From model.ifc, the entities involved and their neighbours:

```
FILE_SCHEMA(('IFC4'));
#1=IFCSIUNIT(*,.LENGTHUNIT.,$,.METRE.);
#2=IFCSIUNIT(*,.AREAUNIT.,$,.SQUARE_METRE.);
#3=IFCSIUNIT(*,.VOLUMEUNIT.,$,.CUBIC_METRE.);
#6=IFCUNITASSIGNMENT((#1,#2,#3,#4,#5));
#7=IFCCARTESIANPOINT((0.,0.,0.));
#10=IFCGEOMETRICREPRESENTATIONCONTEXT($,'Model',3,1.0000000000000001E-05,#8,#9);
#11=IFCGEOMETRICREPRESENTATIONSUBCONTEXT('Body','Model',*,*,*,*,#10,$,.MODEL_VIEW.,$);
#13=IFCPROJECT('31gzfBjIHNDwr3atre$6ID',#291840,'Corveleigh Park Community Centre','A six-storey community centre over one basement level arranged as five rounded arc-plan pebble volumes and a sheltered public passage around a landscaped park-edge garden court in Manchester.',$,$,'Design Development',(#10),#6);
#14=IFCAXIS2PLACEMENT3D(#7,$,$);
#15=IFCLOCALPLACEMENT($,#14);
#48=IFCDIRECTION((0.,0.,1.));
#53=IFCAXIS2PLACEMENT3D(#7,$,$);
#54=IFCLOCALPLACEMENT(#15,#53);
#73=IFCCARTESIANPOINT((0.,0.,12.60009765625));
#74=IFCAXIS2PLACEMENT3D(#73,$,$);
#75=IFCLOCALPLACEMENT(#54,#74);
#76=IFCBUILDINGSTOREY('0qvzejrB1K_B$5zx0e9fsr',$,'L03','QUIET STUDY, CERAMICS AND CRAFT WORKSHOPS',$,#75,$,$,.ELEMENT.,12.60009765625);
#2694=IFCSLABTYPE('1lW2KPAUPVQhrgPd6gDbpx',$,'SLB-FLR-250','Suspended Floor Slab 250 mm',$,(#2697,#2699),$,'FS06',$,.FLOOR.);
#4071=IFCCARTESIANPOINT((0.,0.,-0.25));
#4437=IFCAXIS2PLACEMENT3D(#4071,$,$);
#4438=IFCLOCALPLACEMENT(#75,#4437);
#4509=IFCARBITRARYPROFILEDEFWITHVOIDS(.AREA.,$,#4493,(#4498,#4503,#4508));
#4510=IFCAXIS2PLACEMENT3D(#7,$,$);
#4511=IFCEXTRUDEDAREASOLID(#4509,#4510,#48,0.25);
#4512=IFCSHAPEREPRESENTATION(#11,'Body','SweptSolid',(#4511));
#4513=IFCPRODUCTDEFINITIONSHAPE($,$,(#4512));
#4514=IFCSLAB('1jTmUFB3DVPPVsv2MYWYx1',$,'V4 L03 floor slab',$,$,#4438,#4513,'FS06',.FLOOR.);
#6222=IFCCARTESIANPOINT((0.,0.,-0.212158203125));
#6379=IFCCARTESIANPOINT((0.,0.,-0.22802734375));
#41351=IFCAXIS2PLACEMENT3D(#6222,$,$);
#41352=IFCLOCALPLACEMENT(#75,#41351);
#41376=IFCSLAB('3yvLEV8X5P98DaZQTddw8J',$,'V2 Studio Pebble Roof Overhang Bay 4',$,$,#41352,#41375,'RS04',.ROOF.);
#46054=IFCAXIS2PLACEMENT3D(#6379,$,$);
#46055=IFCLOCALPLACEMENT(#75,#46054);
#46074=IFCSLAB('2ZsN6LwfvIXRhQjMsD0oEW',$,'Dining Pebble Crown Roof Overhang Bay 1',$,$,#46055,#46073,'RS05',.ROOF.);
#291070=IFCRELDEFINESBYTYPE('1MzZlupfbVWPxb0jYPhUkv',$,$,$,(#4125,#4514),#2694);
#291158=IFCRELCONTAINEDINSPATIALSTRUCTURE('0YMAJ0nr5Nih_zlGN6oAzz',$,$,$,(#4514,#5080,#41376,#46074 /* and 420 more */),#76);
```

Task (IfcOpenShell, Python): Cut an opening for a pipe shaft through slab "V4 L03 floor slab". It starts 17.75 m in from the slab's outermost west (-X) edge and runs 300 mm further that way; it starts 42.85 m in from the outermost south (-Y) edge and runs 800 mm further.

```python
import numpy as np
import ifcopenshell
import ifcopenshell.api.feature
import ifcopenshell.api.geometry
import ifcopenshell.api.root
import ifcopenshell.geom
import ifcopenshell.util.placement
import ifcopenshell.util.representation
import ifcopenshell.util.shape
import ifcopenshell.util.unit

model = ifcopenshell.open("model.ifc")
unit_scale = ifcopenshell.util.unit.calculate_unit_scale(model)
settings = ifcopenshell.geom.settings()


def volume(element):
    """Net volume in cubic metres, openings subtracted."""
    shape = ifcopenshell.geom.create_shape(settings, element)
    return ifcopenshell.util.shape.get_volume(shape.geometry)


slab = model.by_guid("1jTmUFB3DVPPVsv2MYWYx1")
before = volume(slab)

# Extent in the slab's own axes, in metres. The edges named are its -X and -Y sides.
slab_shape = ifcopenshell.geom.create_shape(settings, slab)
vertices = ifcopenshell.util.shape.get_vertices(slab_shape.geometry)
x_min, y_min, bottom = vertices.min(axis=0)
top = vertices[:, 2].max()

opening = ifcopenshell.api.root.create_entity(model, ifc_class="IfcOpeningElement", name="Pipe shaft opening", predefined_type="OPENING")
context = ifcopenshell.util.representation.get_context(model, "Model", "Body", "MODEL_VIEW")
width, depth = 0.3, 0.8
outline = [(0.0, 0.0), (width, 0.0), (width, depth), (0.0, depth), (0.0, 0.0)]
# Overshoot both faces by 50 mm so the cut is clean.
shape = ifcopenshell.api.geometry.add_slab_representation(
    model, context=context, depth=top - bottom + 0.1, polyline=outline
)
ifcopenshell.api.geometry.assign_representation(model, product=opening, representation=shape)

matrix = ifcopenshell.util.placement.get_local_placement(slab.ObjectPlacement)
matrix[:, 3] = matrix @ np.append(np.array([x_min + 17.75, y_min + 42.85, bottom - 0.05]) / unit_scale, 1.0)
ifcopenshell.api.geometry.edit_object_placement(model, product=opening, matrix=matrix, is_si=False)
ifcopenshell.api.feature.add_feature(model, feature=opening, element=slab)

after = volume(slab)

print(f"slab volume {before:.3f} -> {after:.3f} m3")

model.write("model_v2.ifc")
```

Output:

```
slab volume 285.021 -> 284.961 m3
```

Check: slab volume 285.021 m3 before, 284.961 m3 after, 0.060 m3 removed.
